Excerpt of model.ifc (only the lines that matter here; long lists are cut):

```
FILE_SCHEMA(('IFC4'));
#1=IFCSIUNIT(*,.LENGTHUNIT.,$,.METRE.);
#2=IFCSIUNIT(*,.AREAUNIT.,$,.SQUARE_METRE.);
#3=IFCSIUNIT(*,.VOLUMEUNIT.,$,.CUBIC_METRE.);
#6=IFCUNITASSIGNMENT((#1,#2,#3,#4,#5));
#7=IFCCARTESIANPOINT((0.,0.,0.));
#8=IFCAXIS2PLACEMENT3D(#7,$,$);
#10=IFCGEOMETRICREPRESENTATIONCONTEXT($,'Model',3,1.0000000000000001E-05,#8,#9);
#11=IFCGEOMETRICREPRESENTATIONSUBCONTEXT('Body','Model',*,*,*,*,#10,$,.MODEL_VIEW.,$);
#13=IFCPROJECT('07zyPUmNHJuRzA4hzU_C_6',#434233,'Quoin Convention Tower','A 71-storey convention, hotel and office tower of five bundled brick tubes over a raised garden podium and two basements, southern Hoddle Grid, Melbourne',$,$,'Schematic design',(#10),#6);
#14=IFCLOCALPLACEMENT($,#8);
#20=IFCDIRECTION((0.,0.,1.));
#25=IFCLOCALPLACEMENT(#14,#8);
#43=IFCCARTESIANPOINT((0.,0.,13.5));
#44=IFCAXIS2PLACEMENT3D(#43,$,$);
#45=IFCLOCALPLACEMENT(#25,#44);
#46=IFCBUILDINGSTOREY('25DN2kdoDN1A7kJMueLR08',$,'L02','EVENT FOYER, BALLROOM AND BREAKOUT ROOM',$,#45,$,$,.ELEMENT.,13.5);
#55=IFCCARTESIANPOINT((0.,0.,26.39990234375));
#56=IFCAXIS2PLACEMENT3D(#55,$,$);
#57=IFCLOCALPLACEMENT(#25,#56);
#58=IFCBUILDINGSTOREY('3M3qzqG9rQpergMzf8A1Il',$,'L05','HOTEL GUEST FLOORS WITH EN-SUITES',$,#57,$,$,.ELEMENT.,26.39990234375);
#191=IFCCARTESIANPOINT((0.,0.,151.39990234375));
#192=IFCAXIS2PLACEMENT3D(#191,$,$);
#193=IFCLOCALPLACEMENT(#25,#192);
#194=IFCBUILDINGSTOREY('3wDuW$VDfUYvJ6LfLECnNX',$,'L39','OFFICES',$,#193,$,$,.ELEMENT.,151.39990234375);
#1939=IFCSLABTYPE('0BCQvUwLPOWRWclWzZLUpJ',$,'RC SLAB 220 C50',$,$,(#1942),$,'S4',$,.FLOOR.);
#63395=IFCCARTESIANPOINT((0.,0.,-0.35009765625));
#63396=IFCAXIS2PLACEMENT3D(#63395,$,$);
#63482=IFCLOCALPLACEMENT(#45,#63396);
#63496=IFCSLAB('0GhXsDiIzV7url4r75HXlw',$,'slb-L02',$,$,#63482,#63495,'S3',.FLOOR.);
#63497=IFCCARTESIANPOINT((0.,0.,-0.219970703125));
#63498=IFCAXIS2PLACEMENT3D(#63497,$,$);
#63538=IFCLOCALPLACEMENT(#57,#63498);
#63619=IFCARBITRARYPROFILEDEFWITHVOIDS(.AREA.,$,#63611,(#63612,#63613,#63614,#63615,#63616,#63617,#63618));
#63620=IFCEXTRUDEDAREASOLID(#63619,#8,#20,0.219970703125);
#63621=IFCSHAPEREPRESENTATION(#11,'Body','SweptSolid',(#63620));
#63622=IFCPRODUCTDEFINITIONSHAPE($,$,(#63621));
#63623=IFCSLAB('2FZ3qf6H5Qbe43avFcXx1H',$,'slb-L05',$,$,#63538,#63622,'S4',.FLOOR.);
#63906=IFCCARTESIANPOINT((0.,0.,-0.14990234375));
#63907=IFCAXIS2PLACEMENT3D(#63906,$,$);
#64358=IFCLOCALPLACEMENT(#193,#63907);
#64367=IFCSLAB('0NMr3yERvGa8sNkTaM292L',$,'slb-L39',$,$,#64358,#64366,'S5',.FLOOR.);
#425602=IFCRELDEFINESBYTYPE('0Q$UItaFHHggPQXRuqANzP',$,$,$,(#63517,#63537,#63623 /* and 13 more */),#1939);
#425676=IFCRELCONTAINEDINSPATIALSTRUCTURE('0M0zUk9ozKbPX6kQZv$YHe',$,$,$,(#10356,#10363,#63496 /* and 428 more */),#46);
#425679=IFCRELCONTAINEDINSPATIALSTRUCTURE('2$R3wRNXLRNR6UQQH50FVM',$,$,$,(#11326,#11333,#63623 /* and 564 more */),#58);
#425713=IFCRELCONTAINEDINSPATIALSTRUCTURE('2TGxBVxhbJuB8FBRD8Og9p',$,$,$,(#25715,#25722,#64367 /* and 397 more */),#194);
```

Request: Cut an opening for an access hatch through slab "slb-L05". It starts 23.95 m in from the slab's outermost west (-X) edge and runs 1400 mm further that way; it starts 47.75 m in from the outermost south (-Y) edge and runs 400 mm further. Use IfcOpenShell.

```python
import numpy as np
import ifcopenshell
import ifcopenshell.api.feature
import ifcopenshell.api.geometry
import ifcopenshell.api.root
import ifcopenshell.geom
import ifcopenshell.util.placement
import ifcopenshell.util.representation
import ifcopenshell.util.shape
import ifcopenshell.util.unit

model = ifcopenshell.open("model.ifc")
unit_scale = ifcopenshell.util.unit.calculate_unit_scale(model)
settings = ifcopenshell.geom.settings()


def volume(element):
    """Net volume in cubic metres, openings subtracted."""
    shape = ifcopenshell.geom.create_shape(settings, element)
    return ifcopenshell.util.shape.get_volume(shape.geometry)


slab = model.by_id(63623)
before = volume(slab)

# Extent in the slab's own axes, in metres. The edges named are its -X and -Y sides.
slab_shape = ifcopenshell.geom.create_shape(settings, slab)
vertices = ifcopenshell.util.shape.get_vertices(slab_shape.geometry)
x_min, y_min, bottom = vertices.min(axis=0)
top = vertices[:, 2].max()

opening = ifcopenshell.api.root.create_entity(model, ifc_class="IfcOpeningElement", name="Access hatch opening", predefined_type="OPENING")
context = ifcopenshell.util.representation.get_context(model, "Model", "Body", "MODEL_VIEW")
width, depth = 1.4, 0.4
outline = [(0.0, 0.0), (width, 0.0), (width, depth), (0.0, depth), (0.0, 0.0)]
# Overshoot both faces by 50 mm so the cut is clean.
shape = ifcopenshell.api.geometry.add_slab_representation(
    model, context=context, depth=top - bottom + 0.1, polyline=outline
)
ifcopenshell.api.geometry.assign_representation(model, product=opening, representation=shape)

matrix = ifcopenshell.util.placement.get_local_placement(slab.ObjectPlacement)
matrix[:, 3] = matrix @ np.append(np.array([x_min + 23.95, y_min + 47.75, bottom - 0.05]) / unit_scale, 1.0)
ifcopenshell.api.geometry.edit_object_placement(model, product=opening, matrix=matrix, is_si=False)
ifcopenshell.api.feature.add_feature(model, feature=opening, element=slab)

after = volume(slab)

print(f"slab volume {before:.3f} -> {after:.3f} m3")

model.write("model_edited.ifc")
```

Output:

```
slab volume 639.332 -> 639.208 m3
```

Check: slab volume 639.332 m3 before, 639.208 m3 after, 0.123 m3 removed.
